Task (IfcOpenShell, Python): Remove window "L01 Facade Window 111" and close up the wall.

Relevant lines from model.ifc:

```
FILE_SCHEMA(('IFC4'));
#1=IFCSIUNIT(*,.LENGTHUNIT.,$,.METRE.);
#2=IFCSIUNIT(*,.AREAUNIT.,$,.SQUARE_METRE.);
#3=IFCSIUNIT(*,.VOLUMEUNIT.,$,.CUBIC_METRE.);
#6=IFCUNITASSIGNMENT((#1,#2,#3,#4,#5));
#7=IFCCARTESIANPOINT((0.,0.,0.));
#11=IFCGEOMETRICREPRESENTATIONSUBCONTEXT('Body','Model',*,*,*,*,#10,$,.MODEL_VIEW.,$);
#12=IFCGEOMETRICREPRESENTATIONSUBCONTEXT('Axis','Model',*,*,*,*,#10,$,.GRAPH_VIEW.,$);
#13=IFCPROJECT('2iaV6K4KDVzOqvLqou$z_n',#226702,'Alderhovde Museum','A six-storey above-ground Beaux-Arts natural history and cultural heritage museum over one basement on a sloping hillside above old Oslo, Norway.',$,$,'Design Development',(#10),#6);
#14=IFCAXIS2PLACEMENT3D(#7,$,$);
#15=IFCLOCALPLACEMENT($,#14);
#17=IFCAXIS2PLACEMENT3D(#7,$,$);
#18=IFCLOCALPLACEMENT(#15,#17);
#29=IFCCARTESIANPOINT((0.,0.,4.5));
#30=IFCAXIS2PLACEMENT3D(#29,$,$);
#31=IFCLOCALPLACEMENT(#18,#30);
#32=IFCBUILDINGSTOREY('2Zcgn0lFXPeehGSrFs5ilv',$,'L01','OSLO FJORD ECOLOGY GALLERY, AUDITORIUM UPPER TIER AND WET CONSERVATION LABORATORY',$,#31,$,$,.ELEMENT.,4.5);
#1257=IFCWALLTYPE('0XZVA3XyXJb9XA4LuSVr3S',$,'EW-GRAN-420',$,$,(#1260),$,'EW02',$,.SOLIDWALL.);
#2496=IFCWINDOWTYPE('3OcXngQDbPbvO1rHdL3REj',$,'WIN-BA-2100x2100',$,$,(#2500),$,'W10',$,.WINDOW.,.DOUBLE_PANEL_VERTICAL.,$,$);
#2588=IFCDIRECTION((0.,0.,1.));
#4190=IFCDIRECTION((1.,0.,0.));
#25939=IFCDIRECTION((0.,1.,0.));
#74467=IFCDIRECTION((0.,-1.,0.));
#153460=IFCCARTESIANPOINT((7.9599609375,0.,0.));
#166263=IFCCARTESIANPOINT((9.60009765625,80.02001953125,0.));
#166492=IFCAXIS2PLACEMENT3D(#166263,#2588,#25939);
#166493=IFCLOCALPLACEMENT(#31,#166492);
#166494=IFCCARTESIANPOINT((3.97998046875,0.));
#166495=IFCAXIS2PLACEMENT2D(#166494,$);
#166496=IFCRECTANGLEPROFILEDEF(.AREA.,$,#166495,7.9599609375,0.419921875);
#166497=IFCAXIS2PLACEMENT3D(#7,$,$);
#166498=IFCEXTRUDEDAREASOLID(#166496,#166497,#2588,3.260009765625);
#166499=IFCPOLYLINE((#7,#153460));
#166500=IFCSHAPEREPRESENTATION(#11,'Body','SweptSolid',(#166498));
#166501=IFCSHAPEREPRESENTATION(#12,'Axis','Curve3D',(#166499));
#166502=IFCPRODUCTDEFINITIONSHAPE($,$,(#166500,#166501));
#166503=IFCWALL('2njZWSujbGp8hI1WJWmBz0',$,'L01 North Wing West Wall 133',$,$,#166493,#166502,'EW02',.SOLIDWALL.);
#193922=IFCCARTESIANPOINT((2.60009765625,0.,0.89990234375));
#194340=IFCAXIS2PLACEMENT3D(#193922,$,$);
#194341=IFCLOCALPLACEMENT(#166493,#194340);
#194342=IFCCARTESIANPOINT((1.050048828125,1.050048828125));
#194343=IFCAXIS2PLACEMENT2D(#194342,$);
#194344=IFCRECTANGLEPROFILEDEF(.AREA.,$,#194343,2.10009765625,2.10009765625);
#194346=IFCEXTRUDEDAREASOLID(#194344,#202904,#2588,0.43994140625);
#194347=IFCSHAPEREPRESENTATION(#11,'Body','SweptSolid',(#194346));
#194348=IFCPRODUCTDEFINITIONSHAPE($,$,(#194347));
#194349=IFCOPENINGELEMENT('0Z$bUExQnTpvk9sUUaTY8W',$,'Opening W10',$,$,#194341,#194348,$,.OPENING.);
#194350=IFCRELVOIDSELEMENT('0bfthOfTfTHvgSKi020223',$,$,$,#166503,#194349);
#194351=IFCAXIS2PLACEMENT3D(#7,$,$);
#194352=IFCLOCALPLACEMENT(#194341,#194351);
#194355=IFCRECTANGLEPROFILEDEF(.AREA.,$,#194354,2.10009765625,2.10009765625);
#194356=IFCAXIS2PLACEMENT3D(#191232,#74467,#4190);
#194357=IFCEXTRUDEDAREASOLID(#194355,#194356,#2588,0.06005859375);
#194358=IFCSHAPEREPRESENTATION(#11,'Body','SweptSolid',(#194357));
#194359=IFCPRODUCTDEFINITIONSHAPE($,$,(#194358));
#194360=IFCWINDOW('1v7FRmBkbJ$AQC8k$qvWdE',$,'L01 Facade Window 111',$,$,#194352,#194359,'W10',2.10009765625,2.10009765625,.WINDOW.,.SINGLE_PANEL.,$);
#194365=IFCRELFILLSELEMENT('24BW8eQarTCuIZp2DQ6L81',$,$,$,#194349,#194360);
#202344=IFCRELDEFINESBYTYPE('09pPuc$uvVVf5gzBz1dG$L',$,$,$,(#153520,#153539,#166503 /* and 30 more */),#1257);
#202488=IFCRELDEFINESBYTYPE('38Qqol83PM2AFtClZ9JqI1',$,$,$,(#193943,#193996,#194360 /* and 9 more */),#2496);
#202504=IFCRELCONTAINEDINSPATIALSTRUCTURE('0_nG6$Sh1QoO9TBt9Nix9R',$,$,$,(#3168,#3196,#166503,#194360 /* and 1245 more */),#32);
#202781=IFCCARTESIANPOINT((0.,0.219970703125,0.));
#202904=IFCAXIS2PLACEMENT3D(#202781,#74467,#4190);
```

```python
import ifcopenshell
import ifcopenshell.api.feature
import ifcopenshell.api.root
import ifcopenshell.geom
import ifcopenshell.util.shape

model = ifcopenshell.open("model.ifc")
settings = ifcopenshell.geom.settings()


def volume(element):
    """Net volume in cubic metres, openings subtracted."""
    shape = ifcopenshell.geom.create_shape(settings, element)
    return ifcopenshell.util.shape.get_volume(shape.geometry)


window = model.by_guid("1v7FRmBkbJ$AQC8k$qvWdE")
opening = window.FillsVoids[0].RelatingOpeningElement
wall = opening.VoidsElements[0].RelatingBuildingElement
before = volume(wall)

ifcopenshell.api.root.remove_product(model, product=window)
ifcopenshell.api.feature.remove_feature(model, feature=opening)

after = volume(wall)

print(f"wall volume {before:.3f} -> {after:.3f} m3")

model.write("model_rev.ifc")
```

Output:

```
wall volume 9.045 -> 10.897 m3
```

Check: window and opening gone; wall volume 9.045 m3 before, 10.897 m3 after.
